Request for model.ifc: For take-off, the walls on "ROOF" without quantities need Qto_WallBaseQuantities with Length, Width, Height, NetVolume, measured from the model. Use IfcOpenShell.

First a look at what the model holds.

```python
import ifcopenshell
import ifcopenshell.util.element
import ifcopenshell.util.unit

model = ifcopenshell.open("model.ifc")
print(model.schema)
for unit_type in ("LENGTHUNIT", "AREAUNIT", "VOLUMEUNIT"):
    print(unit_type, ifcopenshell.util.unit.calculate_unit_scale(model, unit_type))
storey = next(s for s in model.by_type("IfcBuildingStorey") if s.Name == "ROOF")
walls = [e for e in ifcopenshell.util.element.get_decomposition(storey) if e.is_a("IfcWall")]
for e in sorted(walls, key=lambda e: e.id()):
    print(e.id(), e.is_a(), e.Name, list(ifcopenshell.util.element.get_psets(e, qtos_only=True)), sep=" | ")
```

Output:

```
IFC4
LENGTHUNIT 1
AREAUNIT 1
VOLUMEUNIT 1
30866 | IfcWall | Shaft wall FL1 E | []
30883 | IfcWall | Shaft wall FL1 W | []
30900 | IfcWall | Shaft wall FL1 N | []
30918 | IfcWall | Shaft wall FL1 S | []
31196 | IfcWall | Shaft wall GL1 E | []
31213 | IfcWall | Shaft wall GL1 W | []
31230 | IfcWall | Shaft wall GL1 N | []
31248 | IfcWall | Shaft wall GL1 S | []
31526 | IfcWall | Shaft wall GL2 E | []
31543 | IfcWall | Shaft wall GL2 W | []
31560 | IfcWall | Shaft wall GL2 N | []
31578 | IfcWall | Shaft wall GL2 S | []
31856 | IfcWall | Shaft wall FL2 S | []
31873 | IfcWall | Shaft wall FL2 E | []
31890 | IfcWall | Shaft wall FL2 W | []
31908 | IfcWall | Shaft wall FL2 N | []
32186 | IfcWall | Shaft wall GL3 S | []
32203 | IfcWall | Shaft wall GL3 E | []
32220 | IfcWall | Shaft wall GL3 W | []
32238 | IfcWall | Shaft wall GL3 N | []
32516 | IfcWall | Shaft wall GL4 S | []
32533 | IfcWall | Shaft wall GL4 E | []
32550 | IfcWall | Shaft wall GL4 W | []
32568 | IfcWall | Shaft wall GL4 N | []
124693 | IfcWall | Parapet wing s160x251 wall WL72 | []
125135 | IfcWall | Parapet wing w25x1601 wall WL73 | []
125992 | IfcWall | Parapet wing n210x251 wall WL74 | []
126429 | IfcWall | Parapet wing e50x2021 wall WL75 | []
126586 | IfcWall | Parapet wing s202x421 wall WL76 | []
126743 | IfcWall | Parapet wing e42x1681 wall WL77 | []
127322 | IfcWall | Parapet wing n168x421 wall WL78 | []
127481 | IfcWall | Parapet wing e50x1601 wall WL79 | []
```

```python
import ifcopenshell
import ifcopenshell.api.pset
import ifcopenshell.geom
import ifcopenshell.util.element
import ifcopenshell.util.shape
import ifcopenshell.util.unit

model = ifcopenshell.open("model.ifc")
unit_scale = ifcopenshell.util.unit.calculate_unit_scale(model)
volume_scale = ifcopenshell.util.unit.calculate_unit_scale(model, "VOLUMEUNIT")
settings = ifcopenshell.geom.settings()

storey = next(s for s in model.by_type("IfcBuildingStorey") if s.Name == "ROOF")
walls = [e for e in ifcopenshell.util.element.get_decomposition(storey) if e.is_a("IfcWall")]

for e in sorted(walls, key=lambda e: e.id()):
    if ifcopenshell.util.element.get_psets(e, qtos_only=True, should_inherit=False):
        continue
    # Geometry comes back in metres, in the element's own axes.
    shape = ifcopenshell.geom.create_shape(settings, e)
    values = {
        "Length": ifcopenshell.util.shape.get_x(shape.geometry) / unit_scale,
        "Width": ifcopenshell.util.shape.get_y(shape.geometry) / unit_scale,
        "Height": ifcopenshell.util.shape.get_z(shape.geometry) / unit_scale,
        "NetVolume": ifcopenshell.util.shape.get_volume(shape.geometry) / volume_scale,
    }
    qto = ifcopenshell.api.pset.add_qto(model, product=e, name="Qto_WallBaseQuantities")
    ifcopenshell.api.pset.edit_qto(model, qto=qto, properties=values)
    print(e.id(), {k: round(v, 3) for k, v in values.items()})

model.write("model-out.ifc")
```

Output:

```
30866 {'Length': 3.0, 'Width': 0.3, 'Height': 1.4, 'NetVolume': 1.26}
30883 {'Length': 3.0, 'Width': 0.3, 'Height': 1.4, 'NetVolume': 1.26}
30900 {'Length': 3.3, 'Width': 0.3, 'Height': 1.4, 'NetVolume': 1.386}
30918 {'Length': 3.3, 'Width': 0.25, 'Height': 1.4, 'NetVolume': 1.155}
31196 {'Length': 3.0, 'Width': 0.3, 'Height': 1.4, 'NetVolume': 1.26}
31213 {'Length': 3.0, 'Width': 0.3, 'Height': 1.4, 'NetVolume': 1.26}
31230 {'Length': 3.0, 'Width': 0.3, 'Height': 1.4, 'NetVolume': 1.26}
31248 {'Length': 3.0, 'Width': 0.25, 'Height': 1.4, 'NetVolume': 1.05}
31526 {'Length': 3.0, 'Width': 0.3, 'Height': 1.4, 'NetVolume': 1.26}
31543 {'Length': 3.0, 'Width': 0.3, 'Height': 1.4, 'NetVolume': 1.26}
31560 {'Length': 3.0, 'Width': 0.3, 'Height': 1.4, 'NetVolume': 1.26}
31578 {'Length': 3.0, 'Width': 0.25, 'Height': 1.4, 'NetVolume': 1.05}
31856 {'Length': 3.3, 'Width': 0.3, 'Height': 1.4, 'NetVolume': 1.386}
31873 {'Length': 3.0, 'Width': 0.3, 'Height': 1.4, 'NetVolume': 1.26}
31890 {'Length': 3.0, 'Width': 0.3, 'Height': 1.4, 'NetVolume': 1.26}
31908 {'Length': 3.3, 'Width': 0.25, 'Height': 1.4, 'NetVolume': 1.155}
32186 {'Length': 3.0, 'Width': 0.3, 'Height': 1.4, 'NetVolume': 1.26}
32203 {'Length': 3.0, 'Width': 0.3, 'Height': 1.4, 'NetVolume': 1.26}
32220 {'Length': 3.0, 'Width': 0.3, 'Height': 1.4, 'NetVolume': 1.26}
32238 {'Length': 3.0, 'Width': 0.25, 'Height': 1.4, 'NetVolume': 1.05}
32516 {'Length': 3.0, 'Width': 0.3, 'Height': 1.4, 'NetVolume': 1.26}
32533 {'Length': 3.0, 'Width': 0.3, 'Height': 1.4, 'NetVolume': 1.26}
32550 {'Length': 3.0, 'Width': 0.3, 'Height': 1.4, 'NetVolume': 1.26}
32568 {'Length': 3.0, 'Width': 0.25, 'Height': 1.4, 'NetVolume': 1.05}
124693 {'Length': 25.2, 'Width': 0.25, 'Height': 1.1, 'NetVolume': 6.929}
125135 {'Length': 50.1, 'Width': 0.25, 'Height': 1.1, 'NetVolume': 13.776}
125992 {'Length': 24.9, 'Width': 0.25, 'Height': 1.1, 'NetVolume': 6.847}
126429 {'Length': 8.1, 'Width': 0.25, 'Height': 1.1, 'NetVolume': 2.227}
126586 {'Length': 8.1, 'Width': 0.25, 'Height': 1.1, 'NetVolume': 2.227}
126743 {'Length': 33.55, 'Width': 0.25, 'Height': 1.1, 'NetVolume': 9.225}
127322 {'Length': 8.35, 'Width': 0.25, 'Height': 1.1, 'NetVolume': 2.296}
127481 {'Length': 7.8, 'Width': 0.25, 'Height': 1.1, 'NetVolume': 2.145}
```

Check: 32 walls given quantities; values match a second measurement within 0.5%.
